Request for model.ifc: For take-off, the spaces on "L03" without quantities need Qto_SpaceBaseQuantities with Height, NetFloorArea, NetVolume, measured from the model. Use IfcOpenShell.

First a look at what the model holds.

```python
import ifcopenshell
import ifcopenshell.util.element
import ifcopenshell.util.unit

model = ifcopenshell.open("model.ifc")
print(model.schema)
for unit_type in ("LENGTHUNIT", "AREAUNIT", "VOLUMEUNIT"):
    print(unit_type, ifcopenshell.util.unit.calculate_unit_scale(model, unit_type))
storey = next(s for s in model.by_type("IfcBuildingStorey") if s.Name == "L03")
spaces = [e for e in ifcopenshell.util.element.get_decomposition(storey) if e.is_a("IfcSpace")]
for e in sorted(spaces, key=lambda e: e.id()):
    print(e.id(), e.is_a(), e.Name, list(ifcopenshell.util.element.get_psets(e, qtos_only=True)), sep=" | ")
```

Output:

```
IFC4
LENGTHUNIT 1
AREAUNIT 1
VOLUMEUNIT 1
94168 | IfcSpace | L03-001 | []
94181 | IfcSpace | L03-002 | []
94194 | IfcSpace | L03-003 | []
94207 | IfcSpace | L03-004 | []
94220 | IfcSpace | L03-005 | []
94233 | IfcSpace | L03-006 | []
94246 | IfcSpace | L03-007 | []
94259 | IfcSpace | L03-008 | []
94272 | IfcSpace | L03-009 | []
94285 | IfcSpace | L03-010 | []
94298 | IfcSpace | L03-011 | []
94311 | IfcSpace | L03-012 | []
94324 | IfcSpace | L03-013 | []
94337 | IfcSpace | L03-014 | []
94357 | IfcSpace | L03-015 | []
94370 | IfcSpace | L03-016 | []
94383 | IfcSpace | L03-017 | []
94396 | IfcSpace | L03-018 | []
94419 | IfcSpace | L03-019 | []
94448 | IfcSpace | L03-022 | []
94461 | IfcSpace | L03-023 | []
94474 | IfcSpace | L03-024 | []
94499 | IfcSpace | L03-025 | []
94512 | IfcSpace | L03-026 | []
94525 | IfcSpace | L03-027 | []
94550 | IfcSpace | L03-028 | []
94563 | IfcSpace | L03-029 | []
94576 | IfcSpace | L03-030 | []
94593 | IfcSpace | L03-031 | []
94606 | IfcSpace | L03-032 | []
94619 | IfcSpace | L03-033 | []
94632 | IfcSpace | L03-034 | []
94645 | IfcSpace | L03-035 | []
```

```python
import ifcopenshell
import ifcopenshell.api.pset
import ifcopenshell.geom
import ifcopenshell.util.element
import ifcopenshell.util.shape
import ifcopenshell.util.unit

model = ifcopenshell.open("model.ifc")
unit_scale = ifcopenshell.util.unit.calculate_unit_scale(model)
area_scale = ifcopenshell.util.unit.calculate_unit_scale(model, "AREAUNIT")
volume_scale = ifcopenshell.util.unit.calculate_unit_scale(model, "VOLUMEUNIT")
settings = ifcopenshell.geom.settings()

storey = next(s for s in model.by_type("IfcBuildingStorey") if s.Name == "L03")
spaces = [e for e in ifcopenshell.util.element.get_decomposition(storey) if e.is_a("IfcSpace")]

for e in sorted(spaces, key=lambda e: e.id()):
    if ifcopenshell.util.element.get_psets(e, qtos_only=True, should_inherit=False):
        continue
    # Geometry comes back in metres, in the element's own axes.
    shape = ifcopenshell.geom.create_shape(settings, e)
    values = {
        "Height": ifcopenshell.util.shape.get_z(shape.geometry) / unit_scale,
        "NetFloorArea": ifcopenshell.util.shape.get_footprint_area(shape.geometry) / area_scale,
        "NetVolume": ifcopenshell.util.shape.get_volume(shape.geometry) / volume_scale,
    }
    qto = ifcopenshell.api.pset.add_qto(model, product=e, name="Qto_SpaceBaseQuantities")
    ifcopenshell.api.pset.edit_qto(model, qto=qto, properties=values)
    print(e.id(), {k: round(v, 3) for k, v in values.items()})

model.write("model_v2.ifc")
```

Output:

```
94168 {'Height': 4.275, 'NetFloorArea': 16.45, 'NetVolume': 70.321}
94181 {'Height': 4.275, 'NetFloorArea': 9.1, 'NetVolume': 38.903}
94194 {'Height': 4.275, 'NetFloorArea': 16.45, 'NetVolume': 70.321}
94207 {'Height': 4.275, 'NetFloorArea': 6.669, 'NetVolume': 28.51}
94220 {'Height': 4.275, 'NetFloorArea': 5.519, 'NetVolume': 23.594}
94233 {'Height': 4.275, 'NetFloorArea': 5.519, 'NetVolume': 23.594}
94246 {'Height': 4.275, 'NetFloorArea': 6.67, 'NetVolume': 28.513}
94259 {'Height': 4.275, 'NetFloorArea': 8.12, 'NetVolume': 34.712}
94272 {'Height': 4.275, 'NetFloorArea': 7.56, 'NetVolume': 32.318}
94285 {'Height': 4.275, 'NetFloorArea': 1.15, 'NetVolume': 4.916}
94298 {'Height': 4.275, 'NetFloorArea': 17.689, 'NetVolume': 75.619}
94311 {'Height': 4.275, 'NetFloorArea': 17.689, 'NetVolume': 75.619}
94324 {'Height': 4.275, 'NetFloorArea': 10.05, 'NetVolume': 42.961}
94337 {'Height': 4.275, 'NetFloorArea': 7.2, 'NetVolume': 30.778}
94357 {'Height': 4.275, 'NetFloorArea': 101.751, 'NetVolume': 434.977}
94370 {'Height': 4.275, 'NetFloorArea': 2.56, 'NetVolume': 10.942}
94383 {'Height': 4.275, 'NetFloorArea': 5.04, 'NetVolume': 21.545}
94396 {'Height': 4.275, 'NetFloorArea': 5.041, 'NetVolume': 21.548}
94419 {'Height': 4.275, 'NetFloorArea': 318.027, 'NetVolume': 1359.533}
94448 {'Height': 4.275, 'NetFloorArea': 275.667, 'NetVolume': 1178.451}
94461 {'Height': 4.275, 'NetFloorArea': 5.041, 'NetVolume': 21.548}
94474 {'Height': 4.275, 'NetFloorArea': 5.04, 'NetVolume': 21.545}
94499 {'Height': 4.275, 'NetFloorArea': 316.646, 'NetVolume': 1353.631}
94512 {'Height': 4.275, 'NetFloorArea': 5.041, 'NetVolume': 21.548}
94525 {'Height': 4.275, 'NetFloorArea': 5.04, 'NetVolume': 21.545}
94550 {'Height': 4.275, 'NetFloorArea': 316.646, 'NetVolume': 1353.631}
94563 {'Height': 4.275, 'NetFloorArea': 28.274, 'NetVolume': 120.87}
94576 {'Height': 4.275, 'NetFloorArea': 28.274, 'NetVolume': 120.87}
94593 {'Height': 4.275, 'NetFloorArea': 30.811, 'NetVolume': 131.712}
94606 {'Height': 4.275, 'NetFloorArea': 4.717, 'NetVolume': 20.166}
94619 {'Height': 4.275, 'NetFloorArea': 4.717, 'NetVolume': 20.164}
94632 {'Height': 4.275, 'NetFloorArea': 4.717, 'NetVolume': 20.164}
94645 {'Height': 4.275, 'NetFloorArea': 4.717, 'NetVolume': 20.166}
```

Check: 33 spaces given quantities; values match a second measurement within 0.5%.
